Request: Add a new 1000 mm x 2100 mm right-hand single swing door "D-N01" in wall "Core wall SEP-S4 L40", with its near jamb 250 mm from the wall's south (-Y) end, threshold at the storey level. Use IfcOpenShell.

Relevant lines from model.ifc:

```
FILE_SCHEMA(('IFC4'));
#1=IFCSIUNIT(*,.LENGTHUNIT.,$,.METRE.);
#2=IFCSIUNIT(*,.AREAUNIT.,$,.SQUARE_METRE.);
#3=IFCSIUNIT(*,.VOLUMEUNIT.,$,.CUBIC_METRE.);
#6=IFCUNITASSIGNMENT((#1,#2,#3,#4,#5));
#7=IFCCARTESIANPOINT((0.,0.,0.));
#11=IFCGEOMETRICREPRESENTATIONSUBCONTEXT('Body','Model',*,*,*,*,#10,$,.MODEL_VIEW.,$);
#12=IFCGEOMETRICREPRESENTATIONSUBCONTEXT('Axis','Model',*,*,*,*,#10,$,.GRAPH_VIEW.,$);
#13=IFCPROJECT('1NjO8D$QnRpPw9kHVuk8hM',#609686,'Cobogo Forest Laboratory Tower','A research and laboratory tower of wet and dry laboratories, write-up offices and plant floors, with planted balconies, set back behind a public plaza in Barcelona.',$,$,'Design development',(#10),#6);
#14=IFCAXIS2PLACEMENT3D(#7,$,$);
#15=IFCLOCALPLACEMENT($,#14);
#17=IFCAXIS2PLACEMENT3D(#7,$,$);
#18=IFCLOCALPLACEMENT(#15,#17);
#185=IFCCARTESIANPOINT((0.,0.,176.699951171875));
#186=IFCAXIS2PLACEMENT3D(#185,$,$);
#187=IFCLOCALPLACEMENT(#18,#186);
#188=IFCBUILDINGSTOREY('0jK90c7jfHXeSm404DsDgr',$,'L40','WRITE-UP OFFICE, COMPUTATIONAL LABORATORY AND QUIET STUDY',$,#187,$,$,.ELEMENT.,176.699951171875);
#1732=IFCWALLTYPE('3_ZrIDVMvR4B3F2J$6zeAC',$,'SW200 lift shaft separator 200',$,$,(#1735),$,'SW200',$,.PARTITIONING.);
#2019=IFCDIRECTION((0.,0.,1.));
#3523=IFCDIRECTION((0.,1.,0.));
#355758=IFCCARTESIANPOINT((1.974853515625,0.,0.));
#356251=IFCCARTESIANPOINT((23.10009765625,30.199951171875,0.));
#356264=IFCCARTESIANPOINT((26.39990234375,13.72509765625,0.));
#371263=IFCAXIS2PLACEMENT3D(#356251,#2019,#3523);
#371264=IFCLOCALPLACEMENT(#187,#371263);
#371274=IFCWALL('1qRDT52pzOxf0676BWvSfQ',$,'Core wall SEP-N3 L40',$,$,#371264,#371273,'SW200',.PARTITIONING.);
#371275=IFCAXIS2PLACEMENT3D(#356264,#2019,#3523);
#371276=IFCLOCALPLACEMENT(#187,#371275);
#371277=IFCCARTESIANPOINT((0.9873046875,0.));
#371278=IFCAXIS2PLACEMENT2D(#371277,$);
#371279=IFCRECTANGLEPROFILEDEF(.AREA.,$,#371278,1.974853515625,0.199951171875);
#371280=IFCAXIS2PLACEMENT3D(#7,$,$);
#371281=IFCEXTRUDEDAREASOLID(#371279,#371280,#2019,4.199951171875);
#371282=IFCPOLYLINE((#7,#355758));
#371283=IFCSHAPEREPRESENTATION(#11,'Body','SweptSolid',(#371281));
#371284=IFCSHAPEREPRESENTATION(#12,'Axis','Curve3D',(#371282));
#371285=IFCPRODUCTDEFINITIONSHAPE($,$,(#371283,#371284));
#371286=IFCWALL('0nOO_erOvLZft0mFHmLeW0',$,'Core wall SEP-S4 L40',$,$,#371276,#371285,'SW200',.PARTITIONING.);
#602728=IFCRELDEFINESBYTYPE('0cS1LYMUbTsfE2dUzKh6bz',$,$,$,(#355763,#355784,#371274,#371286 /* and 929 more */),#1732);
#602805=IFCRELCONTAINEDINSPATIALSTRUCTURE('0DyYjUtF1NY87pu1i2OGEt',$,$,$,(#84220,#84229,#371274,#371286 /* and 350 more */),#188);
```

```python
import numpy as np
import ifcopenshell
import ifcopenshell.api.feature
import ifcopenshell.api.geometry
import ifcopenshell.api.root
import ifcopenshell.api.spatial
import ifcopenshell.geom
import ifcopenshell.util.element
import ifcopenshell.util.placement
import ifcopenshell.util.representation
import ifcopenshell.util.shape
import ifcopenshell.util.unit

model = ifcopenshell.open("model.ifc")
unit_scale = ifcopenshell.util.unit.calculate_unit_scale(model)
settings = ifcopenshell.geom.settings()


def volume(element):
    """Net volume in cubic metres, openings subtracted."""
    shape = ifcopenshell.geom.create_shape(settings, element)
    return ifcopenshell.util.shape.get_volume(shape.geometry)


wall = model.by_id(371286)
storey = ifcopenshell.util.element.get_container(wall, ifc_class="IfcBuildingStorey")
context = ifcopenshell.util.representation.get_context(model, "Model", "Body", "MODEL_VIEW")
before = volume(wall)

width, height, from_end, sill = 1, 2.1, 0.25, 0.0  # metres

# The wall runs along its own X axis, and the end named is its -X end.
wall_shape = ifcopenshell.geom.create_shape(settings, wall)
x, y, z = ifcopenshell.util.shape.get_vertices(wall_shape.geometry).T
start = x.min() + from_end
face, thickness = float(y.min()), float(y.max() - y.min())
wall_matrix = ifcopenshell.util.placement.get_local_placement(wall.ObjectPlacement)
level = ifcopenshell.util.placement.get_local_placement(storey.ObjectPlacement)[2, 3]


def in_wall(x, y):
    """Placement at x, y metres in the wall's axes, at sill height."""
    matrix = wall_matrix.copy()
    matrix[:, 3] = wall_matrix @ np.array([x / unit_scale, y / unit_scale, 0.0, 1.0])
    matrix[2, 3] = level + sill / unit_scale
    return matrix


# Opening: a box that overshoots both wall faces by 50 mm.
opening = ifcopenshell.api.root.create_entity(model, ifc_class="IfcOpeningElement", predefined_type="OPENING")
box = ifcopenshell.api.geometry.add_wall_representation(
    model, context=context, length=width, height=height, thickness=thickness + 0.1
)
ifcopenshell.api.geometry.assign_representation(model, product=opening, representation=box)
ifcopenshell.api.geometry.edit_object_placement(model, product=opening, matrix=in_wall(start, face - 0.05), is_si=False)
ifcopenshell.api.feature.add_feature(model, feature=opening, element=wall)

door = ifcopenshell.api.root.create_entity(model, ifc_class="IfcDoor", name="D-N01", predefined_type="DOOR")
door.OverallWidth, door.OverallHeight = width / unit_scale, height / unit_scale
door.OperationType = "SINGLE_SWING_RIGHT"
body = ifcopenshell.api.geometry.add_door_representation(
    model,
    context=context,
    overall_width=door.OverallWidth,
    overall_height=door.OverallHeight,
    operation_type="SINGLE_SWING_RIGHT",
    lining_properties={"LiningDepth": thickness / unit_scale, "ThresholdDepth": thickness / unit_scale},
)
ifcopenshell.api.geometry.assign_representation(model, product=door, representation=body)
ifcopenshell.api.spatial.assign_container(model, products=[door], relating_structure=storey)
ifcopenshell.api.feature.add_filling(model, opening=opening, element=door)

# The lining spans the wall, so the door starts at the wall face.
ifcopenshell.api.geometry.edit_object_placement(model, product=door, matrix=in_wall(start, face), is_si=False)

after = volume(wall)

print(f"wall volume {before:.3f} -> {after:.3f} m3")

model.write("model-out.ifc")
```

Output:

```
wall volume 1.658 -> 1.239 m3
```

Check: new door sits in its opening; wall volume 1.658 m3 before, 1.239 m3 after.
